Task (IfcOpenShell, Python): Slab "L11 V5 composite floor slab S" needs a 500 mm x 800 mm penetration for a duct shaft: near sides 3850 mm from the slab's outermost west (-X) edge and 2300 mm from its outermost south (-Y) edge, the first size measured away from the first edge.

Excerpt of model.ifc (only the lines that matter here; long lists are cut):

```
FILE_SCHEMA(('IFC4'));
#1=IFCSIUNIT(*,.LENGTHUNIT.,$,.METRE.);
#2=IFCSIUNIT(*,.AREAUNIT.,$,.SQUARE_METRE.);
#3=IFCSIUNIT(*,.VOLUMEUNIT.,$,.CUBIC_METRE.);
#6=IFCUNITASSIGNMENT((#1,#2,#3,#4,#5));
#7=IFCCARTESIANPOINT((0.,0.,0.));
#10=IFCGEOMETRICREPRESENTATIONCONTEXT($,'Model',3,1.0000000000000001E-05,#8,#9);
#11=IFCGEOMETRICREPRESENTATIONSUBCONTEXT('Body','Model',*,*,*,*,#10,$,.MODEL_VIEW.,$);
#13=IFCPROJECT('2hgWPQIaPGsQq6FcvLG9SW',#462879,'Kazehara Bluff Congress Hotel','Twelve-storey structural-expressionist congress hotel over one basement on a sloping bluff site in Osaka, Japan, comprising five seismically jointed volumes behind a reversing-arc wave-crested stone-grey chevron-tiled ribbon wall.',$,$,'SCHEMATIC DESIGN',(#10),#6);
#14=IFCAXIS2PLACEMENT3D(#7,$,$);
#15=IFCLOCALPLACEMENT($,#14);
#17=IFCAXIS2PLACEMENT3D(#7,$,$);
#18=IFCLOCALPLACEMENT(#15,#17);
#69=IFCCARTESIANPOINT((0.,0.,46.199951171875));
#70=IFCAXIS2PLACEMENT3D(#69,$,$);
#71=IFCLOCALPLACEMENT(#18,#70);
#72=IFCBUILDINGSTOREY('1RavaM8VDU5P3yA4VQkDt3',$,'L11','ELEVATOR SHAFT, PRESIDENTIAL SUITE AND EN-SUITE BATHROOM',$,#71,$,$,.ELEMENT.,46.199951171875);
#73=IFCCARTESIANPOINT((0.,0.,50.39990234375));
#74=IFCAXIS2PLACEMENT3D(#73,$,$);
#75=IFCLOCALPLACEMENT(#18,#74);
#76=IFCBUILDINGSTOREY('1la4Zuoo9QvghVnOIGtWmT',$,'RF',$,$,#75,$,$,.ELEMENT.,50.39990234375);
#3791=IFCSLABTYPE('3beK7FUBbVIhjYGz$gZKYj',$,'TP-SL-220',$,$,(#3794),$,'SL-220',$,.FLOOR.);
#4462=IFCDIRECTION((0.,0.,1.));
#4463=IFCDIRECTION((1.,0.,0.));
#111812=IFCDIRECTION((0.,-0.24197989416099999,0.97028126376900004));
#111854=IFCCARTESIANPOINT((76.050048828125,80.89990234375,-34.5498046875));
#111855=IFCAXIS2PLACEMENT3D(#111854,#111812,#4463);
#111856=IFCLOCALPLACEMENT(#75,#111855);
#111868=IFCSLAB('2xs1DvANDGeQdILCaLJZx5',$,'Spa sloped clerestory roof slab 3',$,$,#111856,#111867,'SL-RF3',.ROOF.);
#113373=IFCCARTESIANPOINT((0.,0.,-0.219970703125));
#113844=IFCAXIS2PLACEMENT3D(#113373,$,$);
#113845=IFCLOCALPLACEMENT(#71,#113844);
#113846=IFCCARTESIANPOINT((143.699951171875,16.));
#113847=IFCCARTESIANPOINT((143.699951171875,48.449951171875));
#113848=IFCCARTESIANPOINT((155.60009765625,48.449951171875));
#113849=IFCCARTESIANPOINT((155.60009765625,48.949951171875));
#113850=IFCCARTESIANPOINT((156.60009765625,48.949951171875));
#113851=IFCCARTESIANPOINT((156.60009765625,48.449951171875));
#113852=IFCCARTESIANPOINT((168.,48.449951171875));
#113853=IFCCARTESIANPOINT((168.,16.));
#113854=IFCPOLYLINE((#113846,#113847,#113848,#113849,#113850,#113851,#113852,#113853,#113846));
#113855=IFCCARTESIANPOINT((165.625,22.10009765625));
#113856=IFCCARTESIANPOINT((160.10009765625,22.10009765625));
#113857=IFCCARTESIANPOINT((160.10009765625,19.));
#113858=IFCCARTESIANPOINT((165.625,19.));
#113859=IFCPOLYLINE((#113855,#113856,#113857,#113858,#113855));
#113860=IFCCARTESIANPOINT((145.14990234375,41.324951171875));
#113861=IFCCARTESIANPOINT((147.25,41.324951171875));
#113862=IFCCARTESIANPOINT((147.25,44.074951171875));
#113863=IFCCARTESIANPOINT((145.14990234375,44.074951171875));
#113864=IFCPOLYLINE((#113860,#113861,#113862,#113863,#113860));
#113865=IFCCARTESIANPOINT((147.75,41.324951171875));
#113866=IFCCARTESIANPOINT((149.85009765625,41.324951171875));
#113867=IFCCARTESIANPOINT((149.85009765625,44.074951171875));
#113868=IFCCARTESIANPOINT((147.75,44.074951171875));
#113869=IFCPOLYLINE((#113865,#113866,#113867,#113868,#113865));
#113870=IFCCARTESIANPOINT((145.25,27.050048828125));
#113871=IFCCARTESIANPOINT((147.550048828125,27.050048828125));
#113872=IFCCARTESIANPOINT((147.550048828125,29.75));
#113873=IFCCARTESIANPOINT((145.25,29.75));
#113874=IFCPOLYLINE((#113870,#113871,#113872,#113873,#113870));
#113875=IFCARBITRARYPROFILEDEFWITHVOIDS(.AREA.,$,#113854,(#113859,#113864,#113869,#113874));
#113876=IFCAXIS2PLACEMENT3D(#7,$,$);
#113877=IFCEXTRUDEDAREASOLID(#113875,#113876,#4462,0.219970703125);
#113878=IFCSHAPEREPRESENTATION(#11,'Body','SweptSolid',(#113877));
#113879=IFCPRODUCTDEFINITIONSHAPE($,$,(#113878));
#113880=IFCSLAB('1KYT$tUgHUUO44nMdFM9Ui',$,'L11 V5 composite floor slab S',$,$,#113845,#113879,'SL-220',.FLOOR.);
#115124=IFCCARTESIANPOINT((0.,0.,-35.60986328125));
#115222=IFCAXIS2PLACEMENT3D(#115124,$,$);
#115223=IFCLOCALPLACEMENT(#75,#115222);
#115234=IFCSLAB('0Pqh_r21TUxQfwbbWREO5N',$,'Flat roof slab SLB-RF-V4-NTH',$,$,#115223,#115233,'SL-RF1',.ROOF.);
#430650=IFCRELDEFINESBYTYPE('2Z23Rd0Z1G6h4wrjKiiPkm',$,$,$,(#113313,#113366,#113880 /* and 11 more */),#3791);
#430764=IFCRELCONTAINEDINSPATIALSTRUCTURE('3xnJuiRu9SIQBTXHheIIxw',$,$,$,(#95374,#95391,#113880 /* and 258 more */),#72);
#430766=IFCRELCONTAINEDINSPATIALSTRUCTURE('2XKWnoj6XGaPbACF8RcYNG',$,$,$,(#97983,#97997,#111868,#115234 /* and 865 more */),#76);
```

```python
import numpy as np
import ifcopenshell
import ifcopenshell.api.feature
import ifcopenshell.api.geometry
import ifcopenshell.api.root
import ifcopenshell.geom
import ifcopenshell.util.placement
import ifcopenshell.util.representation
import ifcopenshell.util.shape
import ifcopenshell.util.unit

model = ifcopenshell.open("model.ifc")
unit_scale = ifcopenshell.util.unit.calculate_unit_scale(model)
settings = ifcopenshell.geom.settings()


def volume(element):
    """Net volume in cubic metres, openings subtracted."""
    shape = ifcopenshell.geom.create_shape(settings, element)
    return ifcopenshell.util.shape.get_volume(shape.geometry)


slab = model.by_id(113880)
before = volume(slab)

# Extent in the slab's own axes, in metres. The edges named are its -X and -Y sides.
slab_shape = ifcopenshell.geom.create_shape(settings, slab)
vertices = ifcopenshell.util.shape.get_vertices(slab_shape.geometry)
x_min, y_min, bottom = vertices.min(axis=0)
top = vertices[:, 2].max()

opening = ifcopenshell.api.root.create_entity(model, ifc_class="IfcOpeningElement", name="Duct shaft opening", predefined_type="OPENING")
context = ifcopenshell.util.representation.get_context(model, "Model", "Body", "MODEL_VIEW")
width, depth = 0.5, 0.8
outline = [(0.0, 0.0), (width, 0.0), (width, depth), (0.0, depth), (0.0, 0.0)]
# Overshoot both faces by 50 mm so the cut is clean.
shape = ifcopenshell.api.geometry.add_slab_representation(
    model, context=context, depth=top - bottom + 0.1, polyline=outline
)
ifcopenshell.api.geometry.assign_representation(model, product=opening, representation=shape)

matrix = ifcopenshell.util.placement.get_local_placement(slab.ObjectPlacement)
matrix[:, 3] = matrix @ np.append(np.array([x_min + 3.85, y_min + 2.3, bottom - 0.05]) / unit_scale, 1.0)
ifcopenshell.api.geometry.edit_object_placement(model, product=opening, matrix=matrix, is_si=False)
ifcopenshell.api.feature.add_feature(model, feature=opening, element=slab)

after = volume(slab)

print(f"slab volume {before:.3f} -> {after:.3f} m3")

model.write("model_edited.ifc")
```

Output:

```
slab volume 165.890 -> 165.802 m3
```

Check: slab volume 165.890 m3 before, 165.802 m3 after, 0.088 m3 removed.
